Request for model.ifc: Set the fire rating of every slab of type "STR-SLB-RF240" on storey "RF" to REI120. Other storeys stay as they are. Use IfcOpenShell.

First a look at what the model holds.

```python
import ifcopenshell
import ifcopenshell.util.element

model = ifcopenshell.open("model.ifc")
print(model.schema)
storey = next(s for s in model.by_type("IfcBuildingStorey") if s.Name == "RF")
slabs = [e for e in ifcopenshell.util.element.get_decomposition(storey) if e.is_a("IfcSlab")]
seen = {}
for e in slabs:
    element_type = ifcopenshell.util.element.get_type(e)
    key = (element_type.Name if element_type != e and element_type else None, ifcopenshell.util.element.get_pset(e, "Pset_SlabCommon", "FireRating"))
    seen[key] = seen.get(key, 0) + 1
for (name, value), count in sorted(seen.items(), key=str):
    print(count, "x", name, "|", value)
```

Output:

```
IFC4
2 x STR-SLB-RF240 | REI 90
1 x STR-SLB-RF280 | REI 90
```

```python
import ifcopenshell
import ifcopenshell.api.pset
import ifcopenshell.util.element

model = ifcopenshell.open("model.ifc")

storey = next(s for s in model.by_type("IfcBuildingStorey") if s.Name == "RF")
slabs = [e for e in ifcopenshell.util.element.get_decomposition(storey) if e.is_a("IfcSlab")]

count = 0
for e in slabs:
    element_type = ifcopenshell.util.element.get_type(e)
    if element_type in (None, e) or element_type.Name != "STR-SLB-RF240":
        continue
    # add_pset returns the element's existing set when there is one.
    pset = ifcopenshell.api.pset.add_pset(model, product=e, name="Pset_SlabCommon")
    ifcopenshell.api.pset.edit_pset(model, pset=pset, properties={"FireRating": "REI120"})
    count += 1

print(count, "slabs updated")

model.write("model_updated.ifc")
```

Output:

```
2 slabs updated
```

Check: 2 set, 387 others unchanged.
